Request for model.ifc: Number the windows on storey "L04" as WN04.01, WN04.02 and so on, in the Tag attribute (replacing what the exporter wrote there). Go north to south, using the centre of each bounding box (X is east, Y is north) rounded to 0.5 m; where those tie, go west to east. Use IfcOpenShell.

First a look at what the model holds.

```python
import ifcopenshell
import ifcopenshell.util.element
import ifcopenshell.util.placement

model = ifcopenshell.open("model.ifc")
print(model.schema)
storey = next(s for s in model.by_type("IfcBuildingStorey") if s.Name == "L04")
windows = [e for e in ifcopenshell.util.element.get_decomposition(storey) if e.is_a("IfcWindow")]
for e in sorted(windows, key=lambda e: e.id()):
    origin = ifcopenshell.util.placement.get_local_placement(e.ObjectPlacement)[:3, 3]
    print(e.id(), e.Tag, e.Name, origin.round(2) + 0.0, sep=" | ")
```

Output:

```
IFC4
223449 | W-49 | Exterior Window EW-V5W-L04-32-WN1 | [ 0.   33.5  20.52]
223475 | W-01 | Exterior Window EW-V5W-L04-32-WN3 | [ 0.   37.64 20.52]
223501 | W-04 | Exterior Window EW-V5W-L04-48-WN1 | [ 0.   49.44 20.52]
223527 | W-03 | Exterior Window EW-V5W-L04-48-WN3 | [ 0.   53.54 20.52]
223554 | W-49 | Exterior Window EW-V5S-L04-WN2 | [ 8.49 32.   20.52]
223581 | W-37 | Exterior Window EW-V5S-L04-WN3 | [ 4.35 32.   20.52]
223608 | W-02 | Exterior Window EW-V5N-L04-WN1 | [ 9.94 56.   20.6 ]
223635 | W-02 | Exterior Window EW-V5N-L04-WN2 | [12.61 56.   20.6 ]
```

```python
import ifcopenshell
import ifcopenshell.geom
import ifcopenshell.util.element
import ifcopenshell.util.shape

model = ifcopenshell.open("model.ifc")
settings = ifcopenshell.geom.settings()
settings.set("use-world-coords", True)


def centre(element):
    shape = ifcopenshell.geom.create_shape(settings, element)
    return ifcopenshell.util.shape.get_bbox_centroid(shape.geometry)


storey = next(s for s in model.by_type("IfcBuildingStorey") if s.Name == "L04")
windows = [e for e in ifcopenshell.util.element.get_decomposition(storey) if e.is_a("IfcWindow")]

# Insertion points can sit at a corner or the storey origin, so sort by the geometry (in metres).
centres = {e: centre(e) for e in windows}
windows.sort(key=lambda e: (-round(centres[e][1] / 0.5), centres[e][0]))

for i, e in enumerate(windows, start=1):
    number = f"WN04.{i:02d}"
    e.Tag = number
    print(e.id(), number)

model.write("model-out.ifc")
```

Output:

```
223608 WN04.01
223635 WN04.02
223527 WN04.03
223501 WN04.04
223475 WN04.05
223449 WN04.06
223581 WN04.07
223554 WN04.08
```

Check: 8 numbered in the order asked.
